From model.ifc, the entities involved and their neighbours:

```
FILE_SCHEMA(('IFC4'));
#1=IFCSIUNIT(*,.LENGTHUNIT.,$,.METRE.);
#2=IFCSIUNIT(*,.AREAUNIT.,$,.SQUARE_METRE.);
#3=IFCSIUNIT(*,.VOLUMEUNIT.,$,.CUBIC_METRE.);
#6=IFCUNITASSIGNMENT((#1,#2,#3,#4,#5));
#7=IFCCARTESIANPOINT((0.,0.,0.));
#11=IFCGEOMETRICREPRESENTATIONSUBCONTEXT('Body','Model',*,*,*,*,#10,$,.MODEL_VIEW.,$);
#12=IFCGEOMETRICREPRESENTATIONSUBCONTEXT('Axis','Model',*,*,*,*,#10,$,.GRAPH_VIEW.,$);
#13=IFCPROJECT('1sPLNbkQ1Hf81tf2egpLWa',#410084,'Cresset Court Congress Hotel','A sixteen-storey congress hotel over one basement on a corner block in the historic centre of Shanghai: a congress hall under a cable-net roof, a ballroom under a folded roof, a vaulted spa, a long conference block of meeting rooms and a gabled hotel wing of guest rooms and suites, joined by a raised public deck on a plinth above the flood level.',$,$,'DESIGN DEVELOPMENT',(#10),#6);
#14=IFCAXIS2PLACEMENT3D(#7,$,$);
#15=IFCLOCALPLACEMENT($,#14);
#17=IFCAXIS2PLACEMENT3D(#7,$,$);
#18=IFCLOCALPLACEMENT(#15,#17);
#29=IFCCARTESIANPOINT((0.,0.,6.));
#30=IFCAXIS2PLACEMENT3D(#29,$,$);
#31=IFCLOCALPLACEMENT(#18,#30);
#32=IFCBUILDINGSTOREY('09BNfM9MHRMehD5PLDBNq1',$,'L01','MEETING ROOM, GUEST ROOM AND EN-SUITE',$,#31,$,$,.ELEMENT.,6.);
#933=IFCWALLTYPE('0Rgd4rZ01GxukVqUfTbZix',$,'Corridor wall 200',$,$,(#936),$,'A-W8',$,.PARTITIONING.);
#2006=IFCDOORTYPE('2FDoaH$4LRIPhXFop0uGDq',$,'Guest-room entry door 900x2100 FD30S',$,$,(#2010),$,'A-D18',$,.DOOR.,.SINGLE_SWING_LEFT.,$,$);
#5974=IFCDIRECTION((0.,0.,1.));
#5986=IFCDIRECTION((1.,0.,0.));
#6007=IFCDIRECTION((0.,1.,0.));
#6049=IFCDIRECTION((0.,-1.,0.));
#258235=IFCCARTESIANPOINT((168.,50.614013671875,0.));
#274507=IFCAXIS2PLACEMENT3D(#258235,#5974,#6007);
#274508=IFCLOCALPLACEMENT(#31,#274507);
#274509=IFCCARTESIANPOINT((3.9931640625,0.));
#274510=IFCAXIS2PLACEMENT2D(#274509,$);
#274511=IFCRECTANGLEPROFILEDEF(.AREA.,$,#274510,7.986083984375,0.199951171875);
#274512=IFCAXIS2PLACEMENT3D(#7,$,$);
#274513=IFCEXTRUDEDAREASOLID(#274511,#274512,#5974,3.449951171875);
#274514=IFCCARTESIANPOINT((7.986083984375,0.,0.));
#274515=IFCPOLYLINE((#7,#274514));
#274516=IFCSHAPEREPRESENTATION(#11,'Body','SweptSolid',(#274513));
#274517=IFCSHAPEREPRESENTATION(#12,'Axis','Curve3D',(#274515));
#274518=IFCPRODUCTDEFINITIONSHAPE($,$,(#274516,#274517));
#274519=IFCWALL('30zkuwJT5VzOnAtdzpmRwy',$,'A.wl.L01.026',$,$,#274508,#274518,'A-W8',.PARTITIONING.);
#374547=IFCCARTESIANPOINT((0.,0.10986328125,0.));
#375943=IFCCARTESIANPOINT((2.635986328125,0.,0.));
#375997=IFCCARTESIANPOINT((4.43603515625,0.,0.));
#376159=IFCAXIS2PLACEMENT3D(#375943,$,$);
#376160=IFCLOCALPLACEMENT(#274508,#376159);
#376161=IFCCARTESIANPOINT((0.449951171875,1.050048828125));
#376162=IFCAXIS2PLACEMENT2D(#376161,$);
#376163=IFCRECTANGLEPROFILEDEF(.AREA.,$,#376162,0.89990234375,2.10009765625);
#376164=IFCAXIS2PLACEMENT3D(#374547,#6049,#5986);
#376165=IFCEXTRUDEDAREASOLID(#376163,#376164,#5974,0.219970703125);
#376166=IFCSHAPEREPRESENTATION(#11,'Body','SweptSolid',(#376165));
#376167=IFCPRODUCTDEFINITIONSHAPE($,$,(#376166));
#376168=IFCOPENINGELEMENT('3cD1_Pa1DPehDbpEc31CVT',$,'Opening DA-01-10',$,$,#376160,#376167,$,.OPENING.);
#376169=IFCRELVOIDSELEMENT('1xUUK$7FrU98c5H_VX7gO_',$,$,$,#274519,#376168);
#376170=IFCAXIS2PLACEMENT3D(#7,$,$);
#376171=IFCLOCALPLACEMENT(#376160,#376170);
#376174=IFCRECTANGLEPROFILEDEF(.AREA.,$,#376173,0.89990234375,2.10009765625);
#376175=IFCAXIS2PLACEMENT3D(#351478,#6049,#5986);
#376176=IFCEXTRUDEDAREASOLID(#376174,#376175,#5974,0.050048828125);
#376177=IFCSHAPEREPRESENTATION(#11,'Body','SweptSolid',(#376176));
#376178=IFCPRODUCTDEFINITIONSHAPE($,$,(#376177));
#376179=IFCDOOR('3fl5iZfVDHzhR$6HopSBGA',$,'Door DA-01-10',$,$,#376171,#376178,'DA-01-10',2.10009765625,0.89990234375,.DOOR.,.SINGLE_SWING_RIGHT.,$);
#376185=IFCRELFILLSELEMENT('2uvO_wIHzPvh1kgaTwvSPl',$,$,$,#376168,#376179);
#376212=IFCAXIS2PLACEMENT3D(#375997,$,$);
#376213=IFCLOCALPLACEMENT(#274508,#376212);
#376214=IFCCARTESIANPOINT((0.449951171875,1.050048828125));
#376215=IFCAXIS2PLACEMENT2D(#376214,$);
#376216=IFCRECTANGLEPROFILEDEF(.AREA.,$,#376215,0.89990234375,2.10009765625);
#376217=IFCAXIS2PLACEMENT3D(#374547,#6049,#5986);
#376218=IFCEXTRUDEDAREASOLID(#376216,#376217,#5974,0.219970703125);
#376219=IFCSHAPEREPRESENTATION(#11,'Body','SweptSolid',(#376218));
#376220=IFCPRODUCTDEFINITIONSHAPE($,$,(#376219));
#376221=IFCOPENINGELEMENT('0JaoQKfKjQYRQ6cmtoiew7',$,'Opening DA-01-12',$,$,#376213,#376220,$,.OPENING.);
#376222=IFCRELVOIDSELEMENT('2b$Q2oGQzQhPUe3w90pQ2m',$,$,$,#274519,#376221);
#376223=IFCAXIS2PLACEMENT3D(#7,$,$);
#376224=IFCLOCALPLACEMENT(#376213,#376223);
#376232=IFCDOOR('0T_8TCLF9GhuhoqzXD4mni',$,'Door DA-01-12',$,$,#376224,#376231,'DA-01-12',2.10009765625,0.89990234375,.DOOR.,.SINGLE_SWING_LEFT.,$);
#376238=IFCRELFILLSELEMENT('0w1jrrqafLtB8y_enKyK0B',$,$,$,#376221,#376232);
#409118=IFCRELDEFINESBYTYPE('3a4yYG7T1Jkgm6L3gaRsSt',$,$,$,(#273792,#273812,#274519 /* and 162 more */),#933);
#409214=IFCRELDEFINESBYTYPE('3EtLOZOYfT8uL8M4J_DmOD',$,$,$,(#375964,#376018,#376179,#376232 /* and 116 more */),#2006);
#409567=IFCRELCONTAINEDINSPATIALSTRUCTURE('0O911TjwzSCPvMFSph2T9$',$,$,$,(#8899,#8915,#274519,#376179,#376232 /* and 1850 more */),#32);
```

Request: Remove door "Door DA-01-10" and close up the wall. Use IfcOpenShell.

```python
import ifcopenshell
import ifcopenshell.api.feature
import ifcopenshell.api.root
import ifcopenshell.geom
import ifcopenshell.util.shape

model = ifcopenshell.open("model.ifc")
settings = ifcopenshell.geom.settings()


def volume(element):
    """Net volume in cubic metres, openings subtracted."""
    shape = ifcopenshell.geom.create_shape(settings, element)
    return ifcopenshell.util.shape.get_volume(shape.geometry)


door = model.by_id(376179)
opening = door.FillsVoids[0].RelatingOpeningElement
wall = opening.VoidsElements[0].RelatingBuildingElement
before = volume(wall)

ifcopenshell.api.root.remove_product(model, product=door)
ifcopenshell.api.feature.remove_feature(model, feature=opening)

after = volume(wall)

print(f"wall volume {before:.3f} -> {after:.3f} m3")

model.write("model_v2.ifc")
```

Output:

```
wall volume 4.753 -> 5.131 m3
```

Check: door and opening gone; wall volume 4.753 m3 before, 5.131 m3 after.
